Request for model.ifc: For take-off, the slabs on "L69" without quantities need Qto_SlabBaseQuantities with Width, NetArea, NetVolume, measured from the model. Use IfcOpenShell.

First a look at what the model holds.

```python
import ifcopenshell
import ifcopenshell.util.element
import ifcopenshell.util.unit

model = ifcopenshell.open("model.ifc")
print(model.schema)
for unit_type in ("LENGTHUNIT", "AREAUNIT", "VOLUMEUNIT"):
    print(unit_type, ifcopenshell.util.unit.calculate_unit_scale(model, unit_type))
storey = next(s for s in model.by_type("IfcBuildingStorey") if s.Name == "L69")
slabs = [e for e in ifcopenshell.util.element.get_decomposition(storey) if e.is_a("IfcSlab")]
for e in sorted(slabs, key=lambda e: e.id()):
    print(e.id(), e.is_a(), e.Name, list(ifcopenshell.util.element.get_psets(e, qtos_only=True)), sep=" | ")
```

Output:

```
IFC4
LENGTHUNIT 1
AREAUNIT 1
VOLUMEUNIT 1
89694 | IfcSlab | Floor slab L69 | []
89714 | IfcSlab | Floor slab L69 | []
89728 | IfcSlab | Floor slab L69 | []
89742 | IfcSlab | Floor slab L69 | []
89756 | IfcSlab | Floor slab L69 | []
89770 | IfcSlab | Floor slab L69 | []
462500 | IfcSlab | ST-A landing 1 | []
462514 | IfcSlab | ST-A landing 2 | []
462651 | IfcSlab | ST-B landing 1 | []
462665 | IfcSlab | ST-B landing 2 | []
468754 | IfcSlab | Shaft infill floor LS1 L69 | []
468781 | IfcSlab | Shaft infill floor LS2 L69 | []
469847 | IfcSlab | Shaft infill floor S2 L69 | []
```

```python
import ifcopenshell
import ifcopenshell.api.pset
import ifcopenshell.geom
import ifcopenshell.util.element
import ifcopenshell.util.shape
import ifcopenshell.util.unit

model = ifcopenshell.open("model.ifc")
unit_scale = ifcopenshell.util.unit.calculate_unit_scale(model)
area_scale = ifcopenshell.util.unit.calculate_unit_scale(model, "AREAUNIT")
volume_scale = ifcopenshell.util.unit.calculate_unit_scale(model, "VOLUMEUNIT")
settings = ifcopenshell.geom.settings()

storey = next(s for s in model.by_type("IfcBuildingStorey") if s.Name == "L69")
slabs = [e for e in ifcopenshell.util.element.get_decomposition(storey) if e.is_a("IfcSlab")]

for e in sorted(slabs, key=lambda e: e.id()):
    if ifcopenshell.util.element.get_psets(e, qtos_only=True, should_inherit=False):
        continue
    # Geometry comes back in metres, in the element's own axes.
    shape = ifcopenshell.geom.create_shape(settings, e)
    values = {
        "Width": ifcopenshell.util.shape.get_z(shape.geometry) / unit_scale,
        "NetArea": ifcopenshell.util.shape.get_footprint_area(shape.geometry) / area_scale,
        "NetVolume": ifcopenshell.util.shape.get_volume(shape.geometry) / volume_scale,
    }
    qto = ifcopenshell.api.pset.add_qto(model, product=e, name="Qto_SlabBaseQuantities")
    ifcopenshell.api.pset.edit_qto(model, qto=qto, properties=values)
    print(e.id(), {k: round(v, 3) for k, v in values.items()})

model.write("model_edited.ifc")
```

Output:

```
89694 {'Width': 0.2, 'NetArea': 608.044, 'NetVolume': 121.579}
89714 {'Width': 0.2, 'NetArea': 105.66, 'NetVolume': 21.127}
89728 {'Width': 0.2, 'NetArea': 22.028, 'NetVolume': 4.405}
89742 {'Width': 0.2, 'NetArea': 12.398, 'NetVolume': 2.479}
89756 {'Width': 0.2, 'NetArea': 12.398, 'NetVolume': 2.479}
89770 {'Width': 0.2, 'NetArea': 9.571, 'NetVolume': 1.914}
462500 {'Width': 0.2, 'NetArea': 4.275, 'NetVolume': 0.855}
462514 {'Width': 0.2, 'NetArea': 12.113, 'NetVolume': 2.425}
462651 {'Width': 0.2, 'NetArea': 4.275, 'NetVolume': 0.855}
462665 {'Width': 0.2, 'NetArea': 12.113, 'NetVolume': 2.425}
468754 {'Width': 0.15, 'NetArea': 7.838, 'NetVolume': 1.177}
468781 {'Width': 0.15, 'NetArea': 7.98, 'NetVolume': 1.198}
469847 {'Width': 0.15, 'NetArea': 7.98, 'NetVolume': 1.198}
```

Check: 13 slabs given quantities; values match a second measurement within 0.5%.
